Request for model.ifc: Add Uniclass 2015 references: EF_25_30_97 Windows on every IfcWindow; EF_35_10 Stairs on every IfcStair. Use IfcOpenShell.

First a look at what the model holds.

```python
import ifcopenshell

model = ifcopenshell.open("model.ifc")
print(model.schema)
print("classifications:", [c.Name for c in model.by_type("IfcClassification")])
for ifc_class in ("IfcDoor", "IfcRoof", "IfcStair", "IfcWall", "IfcWindow"):
    print(ifc_class, len(model.by_type(ifc_class)))
```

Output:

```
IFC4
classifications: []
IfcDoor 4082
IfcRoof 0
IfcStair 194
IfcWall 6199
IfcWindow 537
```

```python
import ifcopenshell
import ifcopenshell.api.classification

model = ifcopenshell.open("model.ifc")

system = ifcopenshell.api.classification.add_classification(model, classification="Uniclass 2015")

codes = {
    "IfcWindow": ("EF_25_30_97", "Windows"),
    "IfcStair": ("EF_35_10", "Stairs"),
}
for ifc_class, (code, name) in codes.items():
    products = model.by_type(ifc_class)
    ifcopenshell.api.classification.add_reference(
        model, products=products, classification=system, identification=code, name=name
    )
    print(code, len(products))

model.write("model_v2.ifc")
```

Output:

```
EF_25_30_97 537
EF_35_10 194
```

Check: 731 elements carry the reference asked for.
